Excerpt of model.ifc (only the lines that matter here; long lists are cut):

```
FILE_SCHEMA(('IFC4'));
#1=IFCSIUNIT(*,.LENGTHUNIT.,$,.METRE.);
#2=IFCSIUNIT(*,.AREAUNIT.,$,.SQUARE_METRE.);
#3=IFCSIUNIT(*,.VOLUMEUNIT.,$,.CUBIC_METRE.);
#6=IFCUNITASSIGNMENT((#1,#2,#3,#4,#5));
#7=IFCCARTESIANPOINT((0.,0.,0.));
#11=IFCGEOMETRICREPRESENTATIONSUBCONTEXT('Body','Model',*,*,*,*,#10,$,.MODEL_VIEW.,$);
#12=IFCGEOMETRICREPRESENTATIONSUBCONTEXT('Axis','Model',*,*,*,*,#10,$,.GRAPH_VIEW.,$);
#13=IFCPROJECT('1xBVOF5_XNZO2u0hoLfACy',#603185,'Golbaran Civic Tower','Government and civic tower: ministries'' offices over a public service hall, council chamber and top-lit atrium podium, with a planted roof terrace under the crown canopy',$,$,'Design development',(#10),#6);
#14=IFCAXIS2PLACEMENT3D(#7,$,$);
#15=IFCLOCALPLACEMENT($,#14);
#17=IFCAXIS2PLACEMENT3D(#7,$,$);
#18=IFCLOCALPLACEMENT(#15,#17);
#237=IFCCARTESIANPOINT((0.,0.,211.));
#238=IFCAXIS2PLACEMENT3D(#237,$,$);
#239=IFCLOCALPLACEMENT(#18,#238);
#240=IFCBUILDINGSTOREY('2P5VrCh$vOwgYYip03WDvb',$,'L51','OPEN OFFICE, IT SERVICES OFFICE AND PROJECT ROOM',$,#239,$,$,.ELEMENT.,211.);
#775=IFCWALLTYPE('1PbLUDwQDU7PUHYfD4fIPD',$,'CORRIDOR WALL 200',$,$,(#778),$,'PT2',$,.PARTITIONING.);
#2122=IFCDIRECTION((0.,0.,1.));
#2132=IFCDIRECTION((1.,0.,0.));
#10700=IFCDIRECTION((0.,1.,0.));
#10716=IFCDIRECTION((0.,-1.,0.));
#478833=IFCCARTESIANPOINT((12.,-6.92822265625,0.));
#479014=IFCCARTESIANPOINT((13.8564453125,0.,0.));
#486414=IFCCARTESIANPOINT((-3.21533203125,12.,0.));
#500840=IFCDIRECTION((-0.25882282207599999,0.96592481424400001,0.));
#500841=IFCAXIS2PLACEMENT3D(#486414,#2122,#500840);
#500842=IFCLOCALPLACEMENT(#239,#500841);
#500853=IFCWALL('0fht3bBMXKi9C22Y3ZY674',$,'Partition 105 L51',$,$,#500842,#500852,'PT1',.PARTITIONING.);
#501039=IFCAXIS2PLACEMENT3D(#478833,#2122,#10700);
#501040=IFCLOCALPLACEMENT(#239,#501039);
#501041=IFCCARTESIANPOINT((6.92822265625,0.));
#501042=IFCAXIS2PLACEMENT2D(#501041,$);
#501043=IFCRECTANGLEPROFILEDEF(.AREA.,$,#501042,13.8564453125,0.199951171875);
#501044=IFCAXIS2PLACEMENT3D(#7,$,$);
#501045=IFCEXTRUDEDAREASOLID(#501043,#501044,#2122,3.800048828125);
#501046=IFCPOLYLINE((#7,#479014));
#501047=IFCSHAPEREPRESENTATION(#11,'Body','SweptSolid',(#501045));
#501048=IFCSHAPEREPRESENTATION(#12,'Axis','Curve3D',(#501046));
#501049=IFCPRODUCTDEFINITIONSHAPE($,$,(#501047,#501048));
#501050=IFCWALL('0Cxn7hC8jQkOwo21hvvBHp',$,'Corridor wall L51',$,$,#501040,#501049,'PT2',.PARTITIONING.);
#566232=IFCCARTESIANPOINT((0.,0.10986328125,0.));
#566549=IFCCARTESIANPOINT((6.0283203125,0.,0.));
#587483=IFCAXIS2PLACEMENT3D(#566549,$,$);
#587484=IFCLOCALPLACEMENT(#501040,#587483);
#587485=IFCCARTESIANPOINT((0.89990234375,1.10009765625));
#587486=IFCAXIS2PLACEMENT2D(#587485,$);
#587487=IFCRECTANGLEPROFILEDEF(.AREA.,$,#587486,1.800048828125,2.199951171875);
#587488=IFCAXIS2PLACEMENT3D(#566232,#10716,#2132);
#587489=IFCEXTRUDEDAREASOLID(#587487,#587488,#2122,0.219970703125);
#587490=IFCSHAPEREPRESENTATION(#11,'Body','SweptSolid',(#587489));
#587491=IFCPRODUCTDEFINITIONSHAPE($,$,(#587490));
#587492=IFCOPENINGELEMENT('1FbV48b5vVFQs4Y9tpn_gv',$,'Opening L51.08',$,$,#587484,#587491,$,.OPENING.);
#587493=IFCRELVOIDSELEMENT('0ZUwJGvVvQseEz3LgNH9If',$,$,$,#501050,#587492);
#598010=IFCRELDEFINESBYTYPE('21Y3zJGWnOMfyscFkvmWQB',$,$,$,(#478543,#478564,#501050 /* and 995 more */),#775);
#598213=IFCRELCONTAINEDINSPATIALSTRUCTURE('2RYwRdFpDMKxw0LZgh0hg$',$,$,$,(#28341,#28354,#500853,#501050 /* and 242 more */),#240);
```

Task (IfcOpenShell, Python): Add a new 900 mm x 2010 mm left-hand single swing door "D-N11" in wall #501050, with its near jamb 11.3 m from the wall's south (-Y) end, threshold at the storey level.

```python
import numpy as np
import ifcopenshell
import ifcopenshell.api.feature
import ifcopenshell.api.geometry
import ifcopenshell.api.root
import ifcopenshell.api.spatial
import ifcopenshell.geom
import ifcopenshell.util.element
import ifcopenshell.util.placement
import ifcopenshell.util.representation
import ifcopenshell.util.shape
import ifcopenshell.util.unit

model = ifcopenshell.open("model.ifc")
unit_scale = ifcopenshell.util.unit.calculate_unit_scale(model)
settings = ifcopenshell.geom.settings()


def volume(element):
    """Net volume in cubic metres, openings subtracted."""
    shape = ifcopenshell.geom.create_shape(settings, element)
    return ifcopenshell.util.shape.get_volume(shape.geometry)


wall = model.by_guid("0Cxn7hC8jQkOwo21hvvBHp")
storey = ifcopenshell.util.element.get_container(wall, ifc_class="IfcBuildingStorey")
context = ifcopenshell.util.representation.get_context(model, "Model", "Body", "MODEL_VIEW")
before = volume(wall)

width, height, from_end, sill = 0.9, 2.01, 11.3, 0.0  # metres

# The wall runs along its own X axis, and the end named is its -X end.
wall_shape = ifcopenshell.geom.create_shape(settings, wall)
x, y, z = ifcopenshell.util.shape.get_vertices(wall_shape.geometry).T
start = x.min() + from_end
face, thickness = float(y.min()), float(y.max() - y.min())
wall_matrix = ifcopenshell.util.placement.get_local_placement(wall.ObjectPlacement)
level = ifcopenshell.util.placement.get_local_placement(storey.ObjectPlacement)[2, 3]


def in_wall(x, y):
    """Placement at x, y metres in the wall's axes, at sill height."""
    matrix = wall_matrix.copy()
    matrix[:, 3] = wall_matrix @ np.array([x / unit_scale, y / unit_scale, 0.0, 1.0])
    matrix[2, 3] = level + sill / unit_scale
    return matrix


# Opening: a box that overshoots both wall faces by 50 mm.
opening = ifcopenshell.api.root.create_entity(model, ifc_class="IfcOpeningElement", predefined_type="OPENING")
box = ifcopenshell.api.geometry.add_wall_representation(
    model, context=context, length=width, height=height, thickness=thickness + 0.1
)
ifcopenshell.api.geometry.assign_representation(model, product=opening, representation=box)
ifcopenshell.api.geometry.edit_object_placement(model, product=opening, matrix=in_wall(start, face - 0.05), is_si=False)
ifcopenshell.api.feature.add_feature(model, feature=opening, element=wall)

door = ifcopenshell.api.root.create_entity(model, ifc_class="IfcDoor", name="D-N11", predefined_type="DOOR")
door.OverallWidth, door.OverallHeight = width / unit_scale, height / unit_scale
door.OperationType = "SINGLE_SWING_LEFT"
body = ifcopenshell.api.geometry.add_door_representation(
    model,
    context=context,
    overall_width=door.OverallWidth,
    overall_height=door.OverallHeight,
    operation_type="SINGLE_SWING_LEFT",
    lining_properties={"LiningDepth": thickness / unit_scale, "ThresholdDepth": thickness / unit_scale},
)
ifcopenshell.api.geometry.assign_representation(model, product=door, representation=body)
ifcopenshell.api.spatial.assign_container(model, products=[door], relating_structure=storey)
ifcopenshell.api.feature.add_filling(model, opening=opening, element=door)

# The lining spans the wall, so the door starts at the wall face.
ifcopenshell.api.geometry.edit_object_placement(model, product=door, matrix=in_wall(start, face), is_si=False)

after = volume(wall)

print(f"wall volume {before:.3f} -> {after:.3f} m3")

model.write("model-out.ifc")
```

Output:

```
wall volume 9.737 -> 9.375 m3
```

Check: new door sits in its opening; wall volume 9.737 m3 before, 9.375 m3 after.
